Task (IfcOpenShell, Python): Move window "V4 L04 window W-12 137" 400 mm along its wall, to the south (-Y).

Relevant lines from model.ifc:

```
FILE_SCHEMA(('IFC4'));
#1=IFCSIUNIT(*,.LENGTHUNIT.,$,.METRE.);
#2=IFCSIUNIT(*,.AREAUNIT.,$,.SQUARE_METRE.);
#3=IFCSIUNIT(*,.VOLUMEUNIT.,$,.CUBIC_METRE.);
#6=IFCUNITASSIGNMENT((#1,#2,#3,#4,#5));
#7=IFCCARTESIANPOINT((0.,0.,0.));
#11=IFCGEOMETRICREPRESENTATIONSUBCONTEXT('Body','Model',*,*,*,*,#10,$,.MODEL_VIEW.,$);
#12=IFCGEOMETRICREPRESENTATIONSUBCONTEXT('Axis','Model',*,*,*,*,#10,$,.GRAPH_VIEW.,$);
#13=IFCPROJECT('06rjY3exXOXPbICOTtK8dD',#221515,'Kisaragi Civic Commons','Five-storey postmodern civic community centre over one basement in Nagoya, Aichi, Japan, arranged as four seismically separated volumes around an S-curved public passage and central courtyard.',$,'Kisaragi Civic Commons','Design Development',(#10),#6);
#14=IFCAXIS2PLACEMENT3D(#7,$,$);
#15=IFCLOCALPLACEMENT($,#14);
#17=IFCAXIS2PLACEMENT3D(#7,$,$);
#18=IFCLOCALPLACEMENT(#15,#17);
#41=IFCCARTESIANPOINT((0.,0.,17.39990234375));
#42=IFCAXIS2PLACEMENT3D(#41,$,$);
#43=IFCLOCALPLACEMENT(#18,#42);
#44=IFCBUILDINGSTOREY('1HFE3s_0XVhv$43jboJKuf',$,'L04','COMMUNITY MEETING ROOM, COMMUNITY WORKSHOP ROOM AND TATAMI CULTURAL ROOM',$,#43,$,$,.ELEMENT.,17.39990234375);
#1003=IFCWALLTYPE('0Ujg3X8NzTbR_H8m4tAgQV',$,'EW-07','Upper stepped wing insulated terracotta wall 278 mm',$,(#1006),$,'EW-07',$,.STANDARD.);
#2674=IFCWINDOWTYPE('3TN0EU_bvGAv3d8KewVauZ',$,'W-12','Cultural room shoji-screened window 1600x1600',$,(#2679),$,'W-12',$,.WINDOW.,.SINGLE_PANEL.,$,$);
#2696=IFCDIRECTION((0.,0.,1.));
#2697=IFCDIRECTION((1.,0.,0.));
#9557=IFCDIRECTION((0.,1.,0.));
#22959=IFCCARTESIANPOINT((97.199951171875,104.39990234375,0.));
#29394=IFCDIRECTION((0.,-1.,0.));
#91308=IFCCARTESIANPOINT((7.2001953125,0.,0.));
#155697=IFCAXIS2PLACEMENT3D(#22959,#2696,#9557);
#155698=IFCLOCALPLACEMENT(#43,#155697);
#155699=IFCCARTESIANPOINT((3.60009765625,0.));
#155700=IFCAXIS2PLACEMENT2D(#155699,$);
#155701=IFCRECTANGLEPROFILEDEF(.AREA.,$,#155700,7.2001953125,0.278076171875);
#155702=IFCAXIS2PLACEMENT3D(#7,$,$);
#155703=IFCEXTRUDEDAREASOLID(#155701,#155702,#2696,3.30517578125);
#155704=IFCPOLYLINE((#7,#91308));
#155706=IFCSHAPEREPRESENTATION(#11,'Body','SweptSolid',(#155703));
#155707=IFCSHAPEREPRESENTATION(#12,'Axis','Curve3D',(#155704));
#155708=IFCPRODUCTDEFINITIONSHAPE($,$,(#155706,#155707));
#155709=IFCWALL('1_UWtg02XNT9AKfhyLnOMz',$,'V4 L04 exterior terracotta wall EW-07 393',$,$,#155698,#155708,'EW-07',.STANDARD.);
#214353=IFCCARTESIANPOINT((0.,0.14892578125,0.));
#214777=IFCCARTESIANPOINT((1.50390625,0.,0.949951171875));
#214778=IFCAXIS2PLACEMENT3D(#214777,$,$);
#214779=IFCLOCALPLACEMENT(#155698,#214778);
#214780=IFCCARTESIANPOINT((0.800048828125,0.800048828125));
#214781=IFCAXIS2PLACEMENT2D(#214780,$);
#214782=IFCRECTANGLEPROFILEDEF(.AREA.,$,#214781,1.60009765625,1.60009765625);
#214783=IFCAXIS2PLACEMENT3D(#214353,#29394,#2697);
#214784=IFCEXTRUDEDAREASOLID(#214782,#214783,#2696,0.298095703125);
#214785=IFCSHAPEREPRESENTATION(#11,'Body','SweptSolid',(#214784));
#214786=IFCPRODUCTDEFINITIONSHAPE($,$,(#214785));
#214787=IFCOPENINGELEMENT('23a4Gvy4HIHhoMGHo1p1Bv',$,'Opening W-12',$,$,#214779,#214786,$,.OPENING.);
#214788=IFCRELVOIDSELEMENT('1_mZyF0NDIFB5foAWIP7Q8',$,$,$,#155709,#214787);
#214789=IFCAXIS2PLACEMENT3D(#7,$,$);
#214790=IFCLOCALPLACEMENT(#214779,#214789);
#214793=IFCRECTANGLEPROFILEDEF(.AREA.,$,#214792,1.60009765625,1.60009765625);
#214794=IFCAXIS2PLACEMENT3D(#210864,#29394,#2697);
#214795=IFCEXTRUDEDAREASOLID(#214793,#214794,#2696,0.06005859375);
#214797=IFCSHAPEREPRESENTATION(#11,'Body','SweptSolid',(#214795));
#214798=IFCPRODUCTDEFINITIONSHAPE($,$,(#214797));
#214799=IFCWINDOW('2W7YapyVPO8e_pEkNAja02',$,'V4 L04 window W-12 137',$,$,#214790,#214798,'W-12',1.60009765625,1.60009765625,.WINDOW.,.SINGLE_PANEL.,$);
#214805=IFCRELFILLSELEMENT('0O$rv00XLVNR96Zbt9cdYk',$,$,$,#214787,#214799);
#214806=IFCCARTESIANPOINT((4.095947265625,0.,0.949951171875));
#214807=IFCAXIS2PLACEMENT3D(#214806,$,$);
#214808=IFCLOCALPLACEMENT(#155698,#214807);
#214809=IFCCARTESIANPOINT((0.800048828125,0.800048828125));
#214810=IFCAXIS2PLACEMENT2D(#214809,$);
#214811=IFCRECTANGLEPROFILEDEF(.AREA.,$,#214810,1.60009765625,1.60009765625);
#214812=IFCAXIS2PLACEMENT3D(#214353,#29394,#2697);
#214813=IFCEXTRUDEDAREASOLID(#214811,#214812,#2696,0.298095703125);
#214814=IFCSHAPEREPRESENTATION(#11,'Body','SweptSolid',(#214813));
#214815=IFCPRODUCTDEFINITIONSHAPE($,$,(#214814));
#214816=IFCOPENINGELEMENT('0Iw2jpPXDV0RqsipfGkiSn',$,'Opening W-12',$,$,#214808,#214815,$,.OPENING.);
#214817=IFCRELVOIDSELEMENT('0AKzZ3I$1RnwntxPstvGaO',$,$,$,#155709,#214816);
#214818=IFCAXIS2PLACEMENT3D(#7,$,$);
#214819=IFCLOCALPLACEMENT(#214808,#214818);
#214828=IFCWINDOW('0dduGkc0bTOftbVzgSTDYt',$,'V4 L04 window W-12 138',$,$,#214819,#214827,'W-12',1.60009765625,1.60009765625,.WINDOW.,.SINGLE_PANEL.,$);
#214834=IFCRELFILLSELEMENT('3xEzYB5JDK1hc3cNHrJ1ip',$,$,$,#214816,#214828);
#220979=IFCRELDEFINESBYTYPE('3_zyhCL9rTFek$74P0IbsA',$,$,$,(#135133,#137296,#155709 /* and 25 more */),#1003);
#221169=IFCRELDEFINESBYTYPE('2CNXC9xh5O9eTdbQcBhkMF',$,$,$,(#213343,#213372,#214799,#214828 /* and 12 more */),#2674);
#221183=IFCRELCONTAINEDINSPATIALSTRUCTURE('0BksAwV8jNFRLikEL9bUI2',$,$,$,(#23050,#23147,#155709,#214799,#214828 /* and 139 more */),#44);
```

```python
import ifcopenshell
import ifcopenshell.api.geometry
import ifcopenshell.util.placement
import ifcopenshell.util.unit

model = ifcopenshell.open("model.ifc")
unit_scale = ifcopenshell.util.unit.calculate_unit_scale(model)

window = model.by_id(214799)
opening = window.FillsVoids[0].RelatingOpeningElement
wall = opening.VoidsElements[0].RelatingBuildingElement

wall_matrix = ifcopenshell.util.placement.get_local_placement(wall.ObjectPlacement)
shift = wall_matrix[:3, 0] * -0.4 / unit_scale
before = ifcopenshell.util.placement.get_local_placement(window.ObjectPlacement)[:3, 3].copy()

# The window is placed relative to its opening, so it follows when the opening moves.
matrix = ifcopenshell.util.placement.get_local_placement(opening.ObjectPlacement)
matrix[:3, 3] += shift
ifcopenshell.api.geometry.edit_object_placement(
    model, product=opening, matrix=matrix, is_si=False, should_transform_children=True
)

after = ifcopenshell.util.placement.get_local_placement(window.ObjectPlacement)[:3, 3]
print("window moved by", (after - before).round(3) + 0.0)

model.write("model_updated.ifc")
```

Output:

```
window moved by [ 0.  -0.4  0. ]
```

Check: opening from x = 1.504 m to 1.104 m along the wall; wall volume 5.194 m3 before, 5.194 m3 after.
